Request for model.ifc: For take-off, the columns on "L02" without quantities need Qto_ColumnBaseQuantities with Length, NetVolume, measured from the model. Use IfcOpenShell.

First a look at what the model holds.

```python
import ifcopenshell
import ifcopenshell.util.element
import ifcopenshell.util.unit

model = ifcopenshell.open("model.ifc")
print(model.schema)
for unit_type in ("LENGTHUNIT", "AREAUNIT", "VOLUMEUNIT"):
    print(unit_type, ifcopenshell.util.unit.calculate_unit_scale(model, unit_type))
storey = next(s for s in model.by_type("IfcBuildingStorey") if s.Name == "L02")
columns = [e for e in ifcopenshell.util.element.get_decomposition(storey) if e.is_a("IfcColumn")]
for e in sorted(columns, key=lambda e: e.id()):
    print(e.id(), e.is_a(), e.Name, list(ifcopenshell.util.element.get_psets(e, qtos_only=True)), sep=" | ")
```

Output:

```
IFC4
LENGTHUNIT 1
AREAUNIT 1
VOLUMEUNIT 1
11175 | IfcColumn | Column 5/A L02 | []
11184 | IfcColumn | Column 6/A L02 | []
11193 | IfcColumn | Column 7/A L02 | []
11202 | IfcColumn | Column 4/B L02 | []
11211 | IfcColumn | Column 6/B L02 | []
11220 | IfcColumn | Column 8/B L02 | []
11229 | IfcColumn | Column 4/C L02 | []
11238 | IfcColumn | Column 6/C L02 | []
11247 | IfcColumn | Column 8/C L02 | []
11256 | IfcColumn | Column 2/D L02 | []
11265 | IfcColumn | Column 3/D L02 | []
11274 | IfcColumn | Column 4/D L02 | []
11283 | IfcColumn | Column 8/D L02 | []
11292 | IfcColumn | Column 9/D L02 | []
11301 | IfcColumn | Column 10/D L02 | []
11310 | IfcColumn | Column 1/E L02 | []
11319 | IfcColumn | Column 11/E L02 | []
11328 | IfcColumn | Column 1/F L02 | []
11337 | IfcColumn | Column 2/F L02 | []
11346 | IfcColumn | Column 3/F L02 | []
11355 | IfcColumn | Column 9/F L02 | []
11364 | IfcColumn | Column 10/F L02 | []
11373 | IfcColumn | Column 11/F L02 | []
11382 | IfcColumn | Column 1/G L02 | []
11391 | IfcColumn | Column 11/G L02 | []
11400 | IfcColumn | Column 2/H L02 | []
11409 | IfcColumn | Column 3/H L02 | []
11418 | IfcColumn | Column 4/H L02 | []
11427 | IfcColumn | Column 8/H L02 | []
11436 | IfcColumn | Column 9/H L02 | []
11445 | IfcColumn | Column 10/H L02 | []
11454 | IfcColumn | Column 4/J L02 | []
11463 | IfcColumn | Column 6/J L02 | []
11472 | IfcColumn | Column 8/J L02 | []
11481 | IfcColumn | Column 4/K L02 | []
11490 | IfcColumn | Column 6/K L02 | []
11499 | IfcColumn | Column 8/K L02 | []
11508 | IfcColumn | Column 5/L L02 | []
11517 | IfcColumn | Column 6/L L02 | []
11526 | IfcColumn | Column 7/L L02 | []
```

```python
import ifcopenshell
import ifcopenshell.api.pset
import ifcopenshell.geom
import ifcopenshell.util.element
import ifcopenshell.util.shape
import ifcopenshell.util.unit

model = ifcopenshell.open("model.ifc")
unit_scale = ifcopenshell.util.unit.calculate_unit_scale(model)
volume_scale = ifcopenshell.util.unit.calculate_unit_scale(model, "VOLUMEUNIT")
settings = ifcopenshell.geom.settings()

storey = next(s for s in model.by_type("IfcBuildingStorey") if s.Name == "L02")
columns = [e for e in ifcopenshell.util.element.get_decomposition(storey) if e.is_a("IfcColumn")]

for e in sorted(columns, key=lambda e: e.id()):
    if ifcopenshell.util.element.get_psets(e, qtos_only=True, should_inherit=False):
        continue
    # Geometry comes back in metres, in the element's own axes.
    shape = ifcopenshell.geom.create_shape(settings, e)
    values = {
        "Length": ifcopenshell.util.shape.get_z(shape.geometry) / unit_scale,
        "NetVolume": ifcopenshell.util.shape.get_volume(shape.geometry) / volume_scale,
    }
    qto = ifcopenshell.api.pset.add_qto(model, product=e, name="Qto_ColumnBaseQuantities")
    ifcopenshell.api.pset.edit_qto(model, qto=qto, properties=values)
    print(e.id(), {k: round(v, 3) for k, v in values.items()})

model.write("model_edited.ifc")
```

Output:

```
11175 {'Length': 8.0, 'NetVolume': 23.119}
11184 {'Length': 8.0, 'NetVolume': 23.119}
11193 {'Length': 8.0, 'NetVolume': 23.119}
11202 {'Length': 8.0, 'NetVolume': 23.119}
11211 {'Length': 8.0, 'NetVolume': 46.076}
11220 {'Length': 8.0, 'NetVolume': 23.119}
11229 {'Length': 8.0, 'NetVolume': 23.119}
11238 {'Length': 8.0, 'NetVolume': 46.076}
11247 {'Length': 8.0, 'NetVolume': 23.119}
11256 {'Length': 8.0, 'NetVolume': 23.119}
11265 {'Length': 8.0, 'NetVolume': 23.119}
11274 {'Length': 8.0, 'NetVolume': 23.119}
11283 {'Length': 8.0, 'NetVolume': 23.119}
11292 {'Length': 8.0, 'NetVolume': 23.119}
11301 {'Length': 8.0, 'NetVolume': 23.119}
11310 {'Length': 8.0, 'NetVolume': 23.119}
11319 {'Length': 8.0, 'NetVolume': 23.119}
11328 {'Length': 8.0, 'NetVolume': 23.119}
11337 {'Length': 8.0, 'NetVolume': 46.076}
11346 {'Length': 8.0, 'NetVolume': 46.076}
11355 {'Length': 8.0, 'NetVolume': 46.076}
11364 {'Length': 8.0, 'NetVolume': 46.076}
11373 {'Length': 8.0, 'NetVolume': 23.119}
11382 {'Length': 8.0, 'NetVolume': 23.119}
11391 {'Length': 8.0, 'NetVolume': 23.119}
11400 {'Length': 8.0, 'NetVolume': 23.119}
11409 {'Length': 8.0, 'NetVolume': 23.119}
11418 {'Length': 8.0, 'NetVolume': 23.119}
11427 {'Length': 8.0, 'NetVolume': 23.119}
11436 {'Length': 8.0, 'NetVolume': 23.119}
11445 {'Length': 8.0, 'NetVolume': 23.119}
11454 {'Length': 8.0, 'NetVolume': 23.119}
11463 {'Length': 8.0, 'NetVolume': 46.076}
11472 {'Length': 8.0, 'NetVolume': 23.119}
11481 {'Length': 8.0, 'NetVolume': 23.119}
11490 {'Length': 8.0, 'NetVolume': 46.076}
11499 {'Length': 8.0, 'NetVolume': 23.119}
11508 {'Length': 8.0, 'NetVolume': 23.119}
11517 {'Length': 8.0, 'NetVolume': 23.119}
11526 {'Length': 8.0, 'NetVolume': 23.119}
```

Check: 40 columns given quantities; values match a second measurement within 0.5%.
